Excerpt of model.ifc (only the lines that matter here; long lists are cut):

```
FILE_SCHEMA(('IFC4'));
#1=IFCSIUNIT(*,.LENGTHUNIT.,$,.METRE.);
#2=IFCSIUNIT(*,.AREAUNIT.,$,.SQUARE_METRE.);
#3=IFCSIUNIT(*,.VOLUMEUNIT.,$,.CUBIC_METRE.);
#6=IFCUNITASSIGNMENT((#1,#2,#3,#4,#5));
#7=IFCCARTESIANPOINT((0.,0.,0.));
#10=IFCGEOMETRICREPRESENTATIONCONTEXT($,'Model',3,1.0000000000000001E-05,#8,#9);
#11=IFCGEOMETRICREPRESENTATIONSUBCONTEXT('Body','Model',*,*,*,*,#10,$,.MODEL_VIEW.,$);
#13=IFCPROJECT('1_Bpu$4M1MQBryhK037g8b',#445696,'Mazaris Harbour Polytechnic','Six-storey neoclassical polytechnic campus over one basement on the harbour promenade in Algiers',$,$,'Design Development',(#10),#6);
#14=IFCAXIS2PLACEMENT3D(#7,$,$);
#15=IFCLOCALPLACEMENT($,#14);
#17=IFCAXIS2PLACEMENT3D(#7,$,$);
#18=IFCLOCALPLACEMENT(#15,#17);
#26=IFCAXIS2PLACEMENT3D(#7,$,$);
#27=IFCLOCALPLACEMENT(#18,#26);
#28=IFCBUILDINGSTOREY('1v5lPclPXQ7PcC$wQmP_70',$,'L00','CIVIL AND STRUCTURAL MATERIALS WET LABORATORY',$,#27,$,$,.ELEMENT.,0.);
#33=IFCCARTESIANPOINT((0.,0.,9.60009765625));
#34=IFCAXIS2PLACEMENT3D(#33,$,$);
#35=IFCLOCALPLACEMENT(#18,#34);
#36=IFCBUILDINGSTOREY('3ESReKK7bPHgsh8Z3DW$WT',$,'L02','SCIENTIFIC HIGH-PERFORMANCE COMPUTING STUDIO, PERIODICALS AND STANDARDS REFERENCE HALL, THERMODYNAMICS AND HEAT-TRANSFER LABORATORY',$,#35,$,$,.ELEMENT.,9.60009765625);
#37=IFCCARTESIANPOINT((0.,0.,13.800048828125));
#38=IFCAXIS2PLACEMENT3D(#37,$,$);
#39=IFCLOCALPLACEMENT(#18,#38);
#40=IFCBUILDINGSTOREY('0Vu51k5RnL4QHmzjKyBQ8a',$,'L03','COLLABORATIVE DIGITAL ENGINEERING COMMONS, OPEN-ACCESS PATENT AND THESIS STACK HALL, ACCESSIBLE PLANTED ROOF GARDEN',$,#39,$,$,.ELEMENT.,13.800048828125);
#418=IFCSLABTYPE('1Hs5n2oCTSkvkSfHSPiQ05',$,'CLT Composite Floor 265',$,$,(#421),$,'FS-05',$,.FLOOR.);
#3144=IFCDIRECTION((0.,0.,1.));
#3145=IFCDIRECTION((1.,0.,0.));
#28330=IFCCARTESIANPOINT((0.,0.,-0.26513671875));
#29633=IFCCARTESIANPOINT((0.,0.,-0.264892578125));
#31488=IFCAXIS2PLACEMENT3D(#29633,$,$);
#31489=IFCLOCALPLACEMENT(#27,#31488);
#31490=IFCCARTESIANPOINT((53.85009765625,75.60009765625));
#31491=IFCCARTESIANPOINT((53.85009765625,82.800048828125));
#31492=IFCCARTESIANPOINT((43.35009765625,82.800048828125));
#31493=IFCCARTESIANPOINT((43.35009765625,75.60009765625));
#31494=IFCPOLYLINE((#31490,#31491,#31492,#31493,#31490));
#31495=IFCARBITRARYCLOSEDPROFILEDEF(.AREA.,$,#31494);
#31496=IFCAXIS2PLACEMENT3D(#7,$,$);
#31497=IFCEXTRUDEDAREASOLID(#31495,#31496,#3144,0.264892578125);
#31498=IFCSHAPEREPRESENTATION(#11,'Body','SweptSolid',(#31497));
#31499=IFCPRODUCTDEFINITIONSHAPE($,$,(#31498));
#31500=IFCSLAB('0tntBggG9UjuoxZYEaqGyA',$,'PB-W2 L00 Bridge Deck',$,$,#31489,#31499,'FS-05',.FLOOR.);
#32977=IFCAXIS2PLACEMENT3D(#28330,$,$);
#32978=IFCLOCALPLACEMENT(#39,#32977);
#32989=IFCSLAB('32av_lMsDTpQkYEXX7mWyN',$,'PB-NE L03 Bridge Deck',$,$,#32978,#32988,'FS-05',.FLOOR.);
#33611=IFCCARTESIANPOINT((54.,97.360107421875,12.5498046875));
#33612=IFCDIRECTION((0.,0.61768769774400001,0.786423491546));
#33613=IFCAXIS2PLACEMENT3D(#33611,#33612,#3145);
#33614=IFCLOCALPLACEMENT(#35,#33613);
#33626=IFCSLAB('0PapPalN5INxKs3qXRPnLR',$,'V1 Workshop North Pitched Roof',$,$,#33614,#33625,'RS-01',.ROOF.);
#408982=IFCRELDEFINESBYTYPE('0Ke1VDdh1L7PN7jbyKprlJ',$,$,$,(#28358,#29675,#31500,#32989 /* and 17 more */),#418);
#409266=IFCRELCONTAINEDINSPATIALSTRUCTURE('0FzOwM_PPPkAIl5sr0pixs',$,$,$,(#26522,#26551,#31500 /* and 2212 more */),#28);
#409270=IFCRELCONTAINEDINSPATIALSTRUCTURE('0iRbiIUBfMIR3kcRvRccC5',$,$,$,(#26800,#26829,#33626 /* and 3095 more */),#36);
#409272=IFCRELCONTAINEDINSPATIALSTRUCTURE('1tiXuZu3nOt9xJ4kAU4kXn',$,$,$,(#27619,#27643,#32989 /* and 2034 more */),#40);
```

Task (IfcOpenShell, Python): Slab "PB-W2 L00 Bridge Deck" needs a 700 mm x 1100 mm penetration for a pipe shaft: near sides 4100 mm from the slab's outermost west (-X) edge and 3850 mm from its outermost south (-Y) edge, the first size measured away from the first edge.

```python
import numpy as np
import ifcopenshell
import ifcopenshell.api.feature
import ifcopenshell.api.geometry
import ifcopenshell.api.root
import ifcopenshell.geom
import ifcopenshell.util.placement
import ifcopenshell.util.representation
import ifcopenshell.util.shape
import ifcopenshell.util.unit

model = ifcopenshell.open("model.ifc")
unit_scale = ifcopenshell.util.unit.calculate_unit_scale(model)
settings = ifcopenshell.geom.settings()


def volume(element):
    """Net volume in cubic metres, openings subtracted."""
    shape = ifcopenshell.geom.create_shape(settings, element)
    return ifcopenshell.util.shape.get_volume(shape.geometry)


slab = model.by_guid("0tntBggG9UjuoxZYEaqGyA")
before = volume(slab)

# Extent in the slab's own axes, in metres. The edges named are its -X and -Y sides.
slab_shape = ifcopenshell.geom.create_shape(settings, slab)
vertices = ifcopenshell.util.shape.get_vertices(slab_shape.geometry)
x_min, y_min, bottom = vertices.min(axis=0)
top = vertices[:, 2].max()

opening = ifcopenshell.api.root.create_entity(model, ifc_class="IfcOpeningElement", name="Pipe shaft opening", predefined_type="OPENING")
context = ifcopenshell.util.representation.get_context(model, "Model", "Body", "MODEL_VIEW")
width, depth = 0.7, 1.1
outline = [(0.0, 0.0), (width, 0.0), (width, depth), (0.0, depth), (0.0, 0.0)]
# Overshoot both faces by 50 mm so the cut is clean.
shape = ifcopenshell.api.geometry.add_slab_representation(
    model, context=context, depth=top - bottom + 0.1, polyline=outline
)
ifcopenshell.api.geometry.assign_representation(model, product=opening, representation=shape)

matrix = ifcopenshell.util.placement.get_local_placement(slab.ObjectPlacement)
matrix[:, 3] = matrix @ np.append(np.array([x_min + 4.1, y_min + 3.85, bottom - 0.05]) / unit_scale, 1.0)
ifcopenshell.api.geometry.edit_object_placement(model, product=opening, matrix=matrix, is_si=False)
ifcopenshell.api.feature.add_feature(model, feature=opening, element=slab)

after = volume(slab)

print(f"slab volume {before:.3f} -> {after:.3f} m3")

model.write("model_updated.ifc")
```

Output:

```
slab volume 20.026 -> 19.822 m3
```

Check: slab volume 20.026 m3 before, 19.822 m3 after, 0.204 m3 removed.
